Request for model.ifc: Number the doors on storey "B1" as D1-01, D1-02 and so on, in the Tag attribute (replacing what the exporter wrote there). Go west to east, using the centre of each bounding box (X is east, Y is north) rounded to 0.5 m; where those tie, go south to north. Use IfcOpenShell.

First a look at what the model holds.

```python
import ifcopenshell
import ifcopenshell.util.element
import ifcopenshell.util.placement

model = ifcopenshell.open("model.ifc")
print(model.schema)
storey = next(s for s in model.by_type("IfcBuildingStorey") if s.Name == "B1")
doors = [e for e in ifcopenshell.util.element.get_decomposition(storey) if e.is_a("IfcDoor")]
for e in sorted(doors, key=lambda e: e.id()):
    origin = ifcopenshell.util.placement.get_local_placement(e.ObjectPlacement)[:3, 3]
    print(e.id(), e.Tag, e.Name, origin.round(2) + 0.0, sep=" | ")
```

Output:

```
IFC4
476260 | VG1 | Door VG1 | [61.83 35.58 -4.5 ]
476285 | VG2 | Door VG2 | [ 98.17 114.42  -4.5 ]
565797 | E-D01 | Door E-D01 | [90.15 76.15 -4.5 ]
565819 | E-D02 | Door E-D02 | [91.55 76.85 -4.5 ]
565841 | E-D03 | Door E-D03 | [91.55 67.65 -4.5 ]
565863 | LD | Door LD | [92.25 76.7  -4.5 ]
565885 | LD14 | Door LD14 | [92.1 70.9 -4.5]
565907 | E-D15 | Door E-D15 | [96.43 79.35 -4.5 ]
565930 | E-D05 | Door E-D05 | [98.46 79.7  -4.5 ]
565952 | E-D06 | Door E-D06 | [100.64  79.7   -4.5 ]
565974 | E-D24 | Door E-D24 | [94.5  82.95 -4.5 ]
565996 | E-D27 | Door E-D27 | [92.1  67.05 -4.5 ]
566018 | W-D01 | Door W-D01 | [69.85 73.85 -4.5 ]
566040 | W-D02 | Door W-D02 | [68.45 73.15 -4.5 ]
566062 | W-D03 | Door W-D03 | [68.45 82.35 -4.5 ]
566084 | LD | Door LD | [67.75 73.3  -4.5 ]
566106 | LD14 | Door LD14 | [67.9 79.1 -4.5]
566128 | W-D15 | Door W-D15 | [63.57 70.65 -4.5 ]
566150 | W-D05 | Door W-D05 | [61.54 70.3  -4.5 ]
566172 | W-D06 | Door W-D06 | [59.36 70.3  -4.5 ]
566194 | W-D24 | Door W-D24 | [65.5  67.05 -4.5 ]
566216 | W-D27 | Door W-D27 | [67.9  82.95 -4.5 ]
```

```python
import ifcopenshell
import ifcopenshell.geom
import ifcopenshell.util.element
import ifcopenshell.util.shape

model = ifcopenshell.open("model.ifc")
settings = ifcopenshell.geom.settings()
settings.set("use-world-coords", True)


def centre(element):
    shape = ifcopenshell.geom.create_shape(settings, element)
    return ifcopenshell.util.shape.get_bbox_centroid(shape.geometry)


storey = next(s for s in model.by_type("IfcBuildingStorey") if s.Name == "B1")
doors = [e for e in ifcopenshell.util.element.get_decomposition(storey) if e.is_a("IfcDoor")]

# Insertion points can sit at a corner or the storey origin, so sort by the geometry (in metres).
centres = {e: centre(e) for e in doors}
doors.sort(key=lambda e: (round(centres[e][0] / 0.5), centres[e][1]))

for i, e in enumerate(doors, start=1):
    number = f"D1-{i:02d}"
    e.Tag = number
    print(e.id(), number)

model.write("model_edited.ifc")
```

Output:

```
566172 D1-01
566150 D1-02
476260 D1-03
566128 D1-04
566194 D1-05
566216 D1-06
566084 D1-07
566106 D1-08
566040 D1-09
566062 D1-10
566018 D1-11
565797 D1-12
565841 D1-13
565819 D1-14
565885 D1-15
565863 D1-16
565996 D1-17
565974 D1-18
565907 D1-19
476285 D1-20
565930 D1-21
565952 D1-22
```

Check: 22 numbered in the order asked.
